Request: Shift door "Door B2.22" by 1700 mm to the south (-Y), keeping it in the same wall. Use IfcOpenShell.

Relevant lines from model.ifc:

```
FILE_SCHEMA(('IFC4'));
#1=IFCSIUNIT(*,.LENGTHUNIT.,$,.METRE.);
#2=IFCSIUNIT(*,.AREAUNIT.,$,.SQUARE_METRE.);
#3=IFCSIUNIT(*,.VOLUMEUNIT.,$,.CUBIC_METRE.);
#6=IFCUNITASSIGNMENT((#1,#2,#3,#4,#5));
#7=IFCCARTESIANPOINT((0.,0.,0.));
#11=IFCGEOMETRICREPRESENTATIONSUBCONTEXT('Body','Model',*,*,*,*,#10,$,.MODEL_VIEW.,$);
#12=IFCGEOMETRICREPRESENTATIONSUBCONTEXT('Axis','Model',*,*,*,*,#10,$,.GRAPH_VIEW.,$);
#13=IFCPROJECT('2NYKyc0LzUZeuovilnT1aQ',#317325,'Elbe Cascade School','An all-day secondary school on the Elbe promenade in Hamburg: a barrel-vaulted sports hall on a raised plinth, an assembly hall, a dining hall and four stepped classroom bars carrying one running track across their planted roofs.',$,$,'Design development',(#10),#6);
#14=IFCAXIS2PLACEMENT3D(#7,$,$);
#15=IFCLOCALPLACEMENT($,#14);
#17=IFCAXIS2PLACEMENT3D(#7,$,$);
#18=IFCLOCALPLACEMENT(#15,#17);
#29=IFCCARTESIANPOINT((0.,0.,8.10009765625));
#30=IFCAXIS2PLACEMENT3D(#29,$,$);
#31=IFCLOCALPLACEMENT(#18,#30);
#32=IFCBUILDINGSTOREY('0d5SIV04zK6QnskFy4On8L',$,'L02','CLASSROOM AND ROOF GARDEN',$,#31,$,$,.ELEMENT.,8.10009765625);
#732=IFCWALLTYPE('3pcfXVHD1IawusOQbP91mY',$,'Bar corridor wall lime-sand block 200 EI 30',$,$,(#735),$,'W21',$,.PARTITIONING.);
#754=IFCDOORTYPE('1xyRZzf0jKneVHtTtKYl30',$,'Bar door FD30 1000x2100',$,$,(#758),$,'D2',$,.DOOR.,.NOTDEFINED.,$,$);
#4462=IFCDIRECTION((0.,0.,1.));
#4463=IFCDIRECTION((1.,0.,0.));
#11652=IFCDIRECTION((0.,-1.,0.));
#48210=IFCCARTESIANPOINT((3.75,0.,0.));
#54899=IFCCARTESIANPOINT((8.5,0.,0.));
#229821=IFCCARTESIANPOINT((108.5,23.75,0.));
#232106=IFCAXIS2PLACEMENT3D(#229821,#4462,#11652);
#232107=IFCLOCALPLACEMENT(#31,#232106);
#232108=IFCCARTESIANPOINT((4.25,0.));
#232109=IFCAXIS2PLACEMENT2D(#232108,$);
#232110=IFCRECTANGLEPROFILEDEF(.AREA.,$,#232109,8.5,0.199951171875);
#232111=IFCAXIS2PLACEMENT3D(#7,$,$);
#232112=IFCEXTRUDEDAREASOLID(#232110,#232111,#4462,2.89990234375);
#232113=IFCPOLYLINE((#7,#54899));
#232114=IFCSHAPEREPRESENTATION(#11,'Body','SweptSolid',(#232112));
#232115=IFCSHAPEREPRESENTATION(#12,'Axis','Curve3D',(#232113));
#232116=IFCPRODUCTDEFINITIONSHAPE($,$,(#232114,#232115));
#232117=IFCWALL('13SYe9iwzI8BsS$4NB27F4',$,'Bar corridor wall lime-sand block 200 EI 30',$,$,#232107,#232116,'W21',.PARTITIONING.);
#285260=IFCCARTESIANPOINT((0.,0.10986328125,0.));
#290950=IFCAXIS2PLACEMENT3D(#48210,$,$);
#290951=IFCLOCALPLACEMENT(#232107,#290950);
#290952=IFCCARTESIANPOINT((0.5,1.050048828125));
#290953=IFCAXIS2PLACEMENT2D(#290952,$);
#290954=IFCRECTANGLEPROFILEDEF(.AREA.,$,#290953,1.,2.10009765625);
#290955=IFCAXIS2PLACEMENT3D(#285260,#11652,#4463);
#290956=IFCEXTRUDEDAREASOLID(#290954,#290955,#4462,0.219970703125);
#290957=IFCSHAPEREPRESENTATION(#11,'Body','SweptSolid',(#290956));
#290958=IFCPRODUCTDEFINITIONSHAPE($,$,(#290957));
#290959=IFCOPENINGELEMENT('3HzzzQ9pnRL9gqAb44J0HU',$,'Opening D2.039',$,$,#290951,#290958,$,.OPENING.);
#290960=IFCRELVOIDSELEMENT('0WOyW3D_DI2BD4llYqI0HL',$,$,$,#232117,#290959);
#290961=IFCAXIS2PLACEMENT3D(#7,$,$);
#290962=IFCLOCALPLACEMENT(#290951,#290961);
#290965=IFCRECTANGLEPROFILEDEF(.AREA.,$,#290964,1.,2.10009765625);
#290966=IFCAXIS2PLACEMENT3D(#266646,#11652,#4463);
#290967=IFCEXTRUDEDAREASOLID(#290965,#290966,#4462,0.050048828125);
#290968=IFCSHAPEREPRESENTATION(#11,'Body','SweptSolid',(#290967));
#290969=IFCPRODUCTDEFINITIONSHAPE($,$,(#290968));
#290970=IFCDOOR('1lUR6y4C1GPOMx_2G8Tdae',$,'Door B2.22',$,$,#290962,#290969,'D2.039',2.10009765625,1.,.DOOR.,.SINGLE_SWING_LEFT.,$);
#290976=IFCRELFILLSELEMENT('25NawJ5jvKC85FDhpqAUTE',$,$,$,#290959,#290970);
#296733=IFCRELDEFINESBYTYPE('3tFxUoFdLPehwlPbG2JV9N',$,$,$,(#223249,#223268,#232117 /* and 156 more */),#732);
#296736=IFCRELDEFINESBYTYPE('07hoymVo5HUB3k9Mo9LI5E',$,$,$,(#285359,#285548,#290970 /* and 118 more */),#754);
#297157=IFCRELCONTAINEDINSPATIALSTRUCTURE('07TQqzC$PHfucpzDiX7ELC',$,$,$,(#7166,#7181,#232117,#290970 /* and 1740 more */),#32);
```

```python
import ifcopenshell
import ifcopenshell.api.geometry
import ifcopenshell.util.placement
import ifcopenshell.util.unit

model = ifcopenshell.open("model.ifc")
unit_scale = ifcopenshell.util.unit.calculate_unit_scale(model)

door = model.by_guid("1lUR6y4C1GPOMx_2G8Tdae")
opening = door.FillsVoids[0].RelatingOpeningElement
wall = opening.VoidsElements[0].RelatingBuildingElement

wall_matrix = ifcopenshell.util.placement.get_local_placement(wall.ObjectPlacement)
shift = wall_matrix[:3, 0] * 1.7 / unit_scale
before = ifcopenshell.util.placement.get_local_placement(door.ObjectPlacement)[:3, 3].copy()

# The door is placed relative to its opening, so it follows when the opening moves.
matrix = ifcopenshell.util.placement.get_local_placement(opening.ObjectPlacement)
matrix[:3, 3] += shift
ifcopenshell.api.geometry.edit_object_placement(
    model, product=opening, matrix=matrix, is_si=False, should_transform_children=True
)

after = ifcopenshell.util.placement.get_local_placement(door.ObjectPlacement)[:3, 3]
print("door moved by", (after - before).round(3) + 0.0)

model.write("model_rev.ifc")
```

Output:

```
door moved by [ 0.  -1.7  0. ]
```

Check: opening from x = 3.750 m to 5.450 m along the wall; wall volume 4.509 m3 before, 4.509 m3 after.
